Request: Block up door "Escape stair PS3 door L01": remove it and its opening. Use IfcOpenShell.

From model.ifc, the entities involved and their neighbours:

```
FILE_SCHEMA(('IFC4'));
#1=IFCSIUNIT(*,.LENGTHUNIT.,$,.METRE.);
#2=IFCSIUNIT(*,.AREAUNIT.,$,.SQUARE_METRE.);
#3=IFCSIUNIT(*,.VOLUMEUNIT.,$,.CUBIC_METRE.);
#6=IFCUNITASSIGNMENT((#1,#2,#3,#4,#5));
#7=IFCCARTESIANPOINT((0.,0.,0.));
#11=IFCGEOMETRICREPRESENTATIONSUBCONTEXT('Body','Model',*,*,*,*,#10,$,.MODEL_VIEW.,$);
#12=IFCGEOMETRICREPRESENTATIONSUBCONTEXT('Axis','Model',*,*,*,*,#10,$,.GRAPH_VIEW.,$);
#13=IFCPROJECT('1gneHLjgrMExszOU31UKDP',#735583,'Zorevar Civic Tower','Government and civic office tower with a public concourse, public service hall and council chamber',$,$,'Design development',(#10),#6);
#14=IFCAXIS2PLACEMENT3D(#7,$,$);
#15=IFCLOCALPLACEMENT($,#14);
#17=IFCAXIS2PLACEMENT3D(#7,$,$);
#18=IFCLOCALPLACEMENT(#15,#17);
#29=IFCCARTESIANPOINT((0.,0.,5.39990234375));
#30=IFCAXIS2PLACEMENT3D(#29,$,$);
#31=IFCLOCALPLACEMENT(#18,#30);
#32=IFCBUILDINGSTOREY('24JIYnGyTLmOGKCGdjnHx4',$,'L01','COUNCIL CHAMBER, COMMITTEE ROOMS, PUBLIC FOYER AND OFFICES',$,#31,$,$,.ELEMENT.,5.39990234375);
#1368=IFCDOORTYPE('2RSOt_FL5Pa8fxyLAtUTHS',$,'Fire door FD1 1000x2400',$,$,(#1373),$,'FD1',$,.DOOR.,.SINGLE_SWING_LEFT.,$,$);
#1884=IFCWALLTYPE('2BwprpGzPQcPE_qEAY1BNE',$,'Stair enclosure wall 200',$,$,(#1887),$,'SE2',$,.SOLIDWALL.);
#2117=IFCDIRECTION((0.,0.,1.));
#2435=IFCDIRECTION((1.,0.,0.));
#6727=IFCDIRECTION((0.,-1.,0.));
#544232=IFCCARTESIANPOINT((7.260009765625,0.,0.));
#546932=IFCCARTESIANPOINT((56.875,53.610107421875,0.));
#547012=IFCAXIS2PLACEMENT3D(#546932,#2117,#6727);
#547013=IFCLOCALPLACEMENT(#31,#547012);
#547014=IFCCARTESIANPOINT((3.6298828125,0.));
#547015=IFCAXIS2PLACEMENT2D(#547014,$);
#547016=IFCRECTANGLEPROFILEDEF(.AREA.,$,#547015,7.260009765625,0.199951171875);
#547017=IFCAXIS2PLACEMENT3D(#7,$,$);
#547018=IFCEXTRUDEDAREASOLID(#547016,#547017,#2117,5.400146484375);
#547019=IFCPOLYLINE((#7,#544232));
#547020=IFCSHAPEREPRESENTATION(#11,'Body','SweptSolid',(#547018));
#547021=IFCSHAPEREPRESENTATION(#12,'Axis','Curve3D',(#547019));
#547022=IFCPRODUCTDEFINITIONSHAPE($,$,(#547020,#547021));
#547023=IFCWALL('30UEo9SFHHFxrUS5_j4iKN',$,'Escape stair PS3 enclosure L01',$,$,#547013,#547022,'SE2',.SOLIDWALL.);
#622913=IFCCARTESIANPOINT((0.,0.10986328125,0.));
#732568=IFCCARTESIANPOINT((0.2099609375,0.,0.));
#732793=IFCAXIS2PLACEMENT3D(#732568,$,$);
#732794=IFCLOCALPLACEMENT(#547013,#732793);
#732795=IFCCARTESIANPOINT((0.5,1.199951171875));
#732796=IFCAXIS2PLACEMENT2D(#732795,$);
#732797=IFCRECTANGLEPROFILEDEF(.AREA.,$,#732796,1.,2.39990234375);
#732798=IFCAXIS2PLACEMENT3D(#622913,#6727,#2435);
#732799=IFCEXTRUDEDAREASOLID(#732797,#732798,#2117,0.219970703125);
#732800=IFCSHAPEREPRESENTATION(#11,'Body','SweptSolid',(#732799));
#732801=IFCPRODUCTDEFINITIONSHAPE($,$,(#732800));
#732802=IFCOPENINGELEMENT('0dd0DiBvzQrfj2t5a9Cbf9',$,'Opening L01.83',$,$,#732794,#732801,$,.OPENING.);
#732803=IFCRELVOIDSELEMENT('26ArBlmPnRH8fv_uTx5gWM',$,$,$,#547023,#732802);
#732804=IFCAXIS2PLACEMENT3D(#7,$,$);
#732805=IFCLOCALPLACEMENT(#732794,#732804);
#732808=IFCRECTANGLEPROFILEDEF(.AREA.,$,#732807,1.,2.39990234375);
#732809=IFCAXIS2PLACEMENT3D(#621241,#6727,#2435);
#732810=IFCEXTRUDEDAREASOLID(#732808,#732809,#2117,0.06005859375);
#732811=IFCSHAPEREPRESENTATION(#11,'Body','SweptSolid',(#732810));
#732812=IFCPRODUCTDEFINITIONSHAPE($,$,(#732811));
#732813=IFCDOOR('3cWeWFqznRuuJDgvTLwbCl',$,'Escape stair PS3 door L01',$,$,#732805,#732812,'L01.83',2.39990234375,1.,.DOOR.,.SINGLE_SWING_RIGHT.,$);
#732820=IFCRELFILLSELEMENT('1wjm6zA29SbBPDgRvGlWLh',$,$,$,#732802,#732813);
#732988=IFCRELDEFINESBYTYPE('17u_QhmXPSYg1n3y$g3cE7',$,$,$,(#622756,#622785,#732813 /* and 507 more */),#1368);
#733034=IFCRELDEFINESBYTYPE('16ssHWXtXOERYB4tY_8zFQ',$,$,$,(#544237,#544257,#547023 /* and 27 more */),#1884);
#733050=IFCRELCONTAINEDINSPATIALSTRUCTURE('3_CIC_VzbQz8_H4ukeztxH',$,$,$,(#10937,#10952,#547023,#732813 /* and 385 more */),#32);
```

```python
import ifcopenshell
import ifcopenshell.api.feature
import ifcopenshell.api.root
import ifcopenshell.geom
import ifcopenshell.util.shape

model = ifcopenshell.open("model.ifc")
settings = ifcopenshell.geom.settings()


def volume(element):
    """Net volume in cubic metres, openings subtracted."""
    shape = ifcopenshell.geom.create_shape(settings, element)
    return ifcopenshell.util.shape.get_volume(shape.geometry)


door = model.by_id(732813)
opening = door.FillsVoids[0].RelatingOpeningElement
wall = opening.VoidsElements[0].RelatingBuildingElement
before = volume(wall)

ifcopenshell.api.root.remove_product(model, product=door)
ifcopenshell.api.feature.remove_feature(model, feature=opening)

after = volume(wall)

print(f"wall volume {before:.3f} -> {after:.3f} m3")

model.write("model_updated.ifc")
```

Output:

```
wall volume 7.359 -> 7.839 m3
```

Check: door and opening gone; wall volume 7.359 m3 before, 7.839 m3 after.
